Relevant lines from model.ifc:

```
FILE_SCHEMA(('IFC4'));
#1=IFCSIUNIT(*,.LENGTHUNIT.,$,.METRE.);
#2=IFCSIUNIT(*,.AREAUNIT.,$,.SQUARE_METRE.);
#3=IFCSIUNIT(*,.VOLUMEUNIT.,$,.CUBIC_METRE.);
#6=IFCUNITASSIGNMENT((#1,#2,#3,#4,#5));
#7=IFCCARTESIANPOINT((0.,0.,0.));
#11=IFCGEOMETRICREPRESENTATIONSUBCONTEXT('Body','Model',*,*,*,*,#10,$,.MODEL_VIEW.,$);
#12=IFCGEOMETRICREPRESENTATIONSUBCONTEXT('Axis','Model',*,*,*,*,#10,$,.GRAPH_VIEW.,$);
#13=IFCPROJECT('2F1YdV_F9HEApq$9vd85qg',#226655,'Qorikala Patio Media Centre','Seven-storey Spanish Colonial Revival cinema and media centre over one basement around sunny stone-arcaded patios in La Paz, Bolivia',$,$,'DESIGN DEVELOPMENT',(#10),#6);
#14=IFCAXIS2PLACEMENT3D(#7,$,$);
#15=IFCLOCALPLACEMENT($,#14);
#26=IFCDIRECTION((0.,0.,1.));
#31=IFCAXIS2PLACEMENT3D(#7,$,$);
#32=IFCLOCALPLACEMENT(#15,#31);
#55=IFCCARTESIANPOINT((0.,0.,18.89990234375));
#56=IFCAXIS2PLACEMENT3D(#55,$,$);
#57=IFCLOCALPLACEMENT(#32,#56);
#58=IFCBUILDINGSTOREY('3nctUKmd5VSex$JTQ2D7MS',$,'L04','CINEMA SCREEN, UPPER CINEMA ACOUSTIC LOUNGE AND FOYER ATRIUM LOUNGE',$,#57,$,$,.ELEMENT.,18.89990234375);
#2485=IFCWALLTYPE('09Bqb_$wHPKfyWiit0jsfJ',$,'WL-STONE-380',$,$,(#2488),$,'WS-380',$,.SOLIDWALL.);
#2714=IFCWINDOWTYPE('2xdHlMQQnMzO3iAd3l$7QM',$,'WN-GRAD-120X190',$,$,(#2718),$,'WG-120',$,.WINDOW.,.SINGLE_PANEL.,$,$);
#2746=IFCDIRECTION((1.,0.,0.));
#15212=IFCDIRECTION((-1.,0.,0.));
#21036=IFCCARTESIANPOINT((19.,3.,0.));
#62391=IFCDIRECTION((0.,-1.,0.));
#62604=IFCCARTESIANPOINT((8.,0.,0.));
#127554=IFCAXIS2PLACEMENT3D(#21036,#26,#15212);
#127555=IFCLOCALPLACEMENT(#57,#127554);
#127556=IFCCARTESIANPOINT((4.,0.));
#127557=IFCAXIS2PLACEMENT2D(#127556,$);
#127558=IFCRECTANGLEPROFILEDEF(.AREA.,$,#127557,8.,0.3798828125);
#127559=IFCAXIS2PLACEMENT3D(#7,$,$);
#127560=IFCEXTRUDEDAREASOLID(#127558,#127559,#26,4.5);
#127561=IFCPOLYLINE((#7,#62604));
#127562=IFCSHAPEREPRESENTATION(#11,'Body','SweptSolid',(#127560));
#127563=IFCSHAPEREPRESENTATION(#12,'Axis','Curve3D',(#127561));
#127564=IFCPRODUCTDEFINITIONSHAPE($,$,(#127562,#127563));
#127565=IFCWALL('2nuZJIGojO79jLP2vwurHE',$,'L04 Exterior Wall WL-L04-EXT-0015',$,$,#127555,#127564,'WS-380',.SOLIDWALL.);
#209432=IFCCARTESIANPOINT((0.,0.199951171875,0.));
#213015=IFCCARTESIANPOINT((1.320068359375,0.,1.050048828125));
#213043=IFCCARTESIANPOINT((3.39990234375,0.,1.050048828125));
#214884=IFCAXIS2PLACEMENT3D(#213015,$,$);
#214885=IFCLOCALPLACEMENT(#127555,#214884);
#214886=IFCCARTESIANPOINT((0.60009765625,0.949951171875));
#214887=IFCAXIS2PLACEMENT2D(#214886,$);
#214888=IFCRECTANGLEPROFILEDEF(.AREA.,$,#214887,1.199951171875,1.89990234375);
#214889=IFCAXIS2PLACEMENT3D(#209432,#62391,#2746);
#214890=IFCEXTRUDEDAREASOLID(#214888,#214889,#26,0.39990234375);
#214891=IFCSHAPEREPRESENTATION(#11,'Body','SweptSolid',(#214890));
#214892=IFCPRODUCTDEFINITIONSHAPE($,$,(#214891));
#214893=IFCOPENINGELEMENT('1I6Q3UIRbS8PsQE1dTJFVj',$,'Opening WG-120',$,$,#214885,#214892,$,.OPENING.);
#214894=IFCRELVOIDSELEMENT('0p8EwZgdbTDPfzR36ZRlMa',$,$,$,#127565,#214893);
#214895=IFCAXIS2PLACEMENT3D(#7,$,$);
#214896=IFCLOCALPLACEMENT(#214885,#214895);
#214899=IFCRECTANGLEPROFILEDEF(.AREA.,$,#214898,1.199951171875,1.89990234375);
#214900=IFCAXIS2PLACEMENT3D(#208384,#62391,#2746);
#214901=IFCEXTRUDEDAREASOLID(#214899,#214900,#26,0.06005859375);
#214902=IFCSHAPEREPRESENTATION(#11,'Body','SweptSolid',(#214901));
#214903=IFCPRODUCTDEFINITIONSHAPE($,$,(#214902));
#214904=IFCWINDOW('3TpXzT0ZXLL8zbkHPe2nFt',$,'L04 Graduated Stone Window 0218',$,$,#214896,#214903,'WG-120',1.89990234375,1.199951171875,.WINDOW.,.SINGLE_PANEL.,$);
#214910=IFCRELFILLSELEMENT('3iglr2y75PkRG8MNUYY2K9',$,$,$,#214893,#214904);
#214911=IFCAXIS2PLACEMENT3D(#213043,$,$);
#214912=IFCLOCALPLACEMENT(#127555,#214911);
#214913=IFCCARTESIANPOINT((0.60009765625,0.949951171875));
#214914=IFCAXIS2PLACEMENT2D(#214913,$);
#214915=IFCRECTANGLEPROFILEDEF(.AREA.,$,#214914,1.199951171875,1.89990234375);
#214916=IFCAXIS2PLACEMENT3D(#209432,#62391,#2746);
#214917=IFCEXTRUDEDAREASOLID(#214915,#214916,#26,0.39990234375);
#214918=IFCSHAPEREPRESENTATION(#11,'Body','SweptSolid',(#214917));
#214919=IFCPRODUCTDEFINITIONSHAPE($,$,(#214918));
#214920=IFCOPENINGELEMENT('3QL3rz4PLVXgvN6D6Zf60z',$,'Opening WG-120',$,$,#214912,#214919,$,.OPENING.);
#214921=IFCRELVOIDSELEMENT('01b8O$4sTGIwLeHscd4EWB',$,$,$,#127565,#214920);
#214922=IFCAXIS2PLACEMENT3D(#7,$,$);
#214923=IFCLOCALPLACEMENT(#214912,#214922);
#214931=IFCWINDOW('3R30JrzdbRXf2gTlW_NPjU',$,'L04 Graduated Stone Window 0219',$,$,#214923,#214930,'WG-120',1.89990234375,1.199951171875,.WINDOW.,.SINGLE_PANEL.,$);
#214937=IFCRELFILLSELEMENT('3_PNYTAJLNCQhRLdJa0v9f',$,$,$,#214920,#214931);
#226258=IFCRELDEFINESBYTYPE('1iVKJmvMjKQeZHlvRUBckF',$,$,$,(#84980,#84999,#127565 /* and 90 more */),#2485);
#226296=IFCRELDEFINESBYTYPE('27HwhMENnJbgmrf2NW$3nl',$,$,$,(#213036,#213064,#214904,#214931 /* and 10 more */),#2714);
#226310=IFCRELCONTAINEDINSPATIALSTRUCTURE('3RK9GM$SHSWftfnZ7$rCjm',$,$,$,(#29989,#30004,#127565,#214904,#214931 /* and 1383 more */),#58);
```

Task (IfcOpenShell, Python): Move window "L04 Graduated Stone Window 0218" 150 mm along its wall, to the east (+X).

```python
import ifcopenshell
import ifcopenshell.api.geometry
import ifcopenshell.util.placement

model = ifcopenshell.open("model.ifc")

window = model.by_id(214904)
opening = window.FillsVoids[0].RelatingOpeningElement
wall = opening.VoidsElements[0].RelatingBuildingElement

wall_matrix = ifcopenshell.util.placement.get_local_placement(wall.ObjectPlacement)
shift = wall_matrix[:3, 0] * -0.15
before = ifcopenshell.util.placement.get_local_placement(window.ObjectPlacement)[:3, 3].copy()

# The window is placed relative to its opening, so it follows when the opening moves.
matrix = ifcopenshell.util.placement.get_local_placement(opening.ObjectPlacement)
matrix[:3, 3] += shift
ifcopenshell.api.geometry.edit_object_placement(
    model, product=opening, matrix=matrix, is_si=False, should_transform_children=True
)

after = ifcopenshell.util.placement.get_local_placement(window.ObjectPlacement)[:3, 3]
print("window moved by", (after - before).round(3) + 0.0)

model.write("model-out.ifc")
```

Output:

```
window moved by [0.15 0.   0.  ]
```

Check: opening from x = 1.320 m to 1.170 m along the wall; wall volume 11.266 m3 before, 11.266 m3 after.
